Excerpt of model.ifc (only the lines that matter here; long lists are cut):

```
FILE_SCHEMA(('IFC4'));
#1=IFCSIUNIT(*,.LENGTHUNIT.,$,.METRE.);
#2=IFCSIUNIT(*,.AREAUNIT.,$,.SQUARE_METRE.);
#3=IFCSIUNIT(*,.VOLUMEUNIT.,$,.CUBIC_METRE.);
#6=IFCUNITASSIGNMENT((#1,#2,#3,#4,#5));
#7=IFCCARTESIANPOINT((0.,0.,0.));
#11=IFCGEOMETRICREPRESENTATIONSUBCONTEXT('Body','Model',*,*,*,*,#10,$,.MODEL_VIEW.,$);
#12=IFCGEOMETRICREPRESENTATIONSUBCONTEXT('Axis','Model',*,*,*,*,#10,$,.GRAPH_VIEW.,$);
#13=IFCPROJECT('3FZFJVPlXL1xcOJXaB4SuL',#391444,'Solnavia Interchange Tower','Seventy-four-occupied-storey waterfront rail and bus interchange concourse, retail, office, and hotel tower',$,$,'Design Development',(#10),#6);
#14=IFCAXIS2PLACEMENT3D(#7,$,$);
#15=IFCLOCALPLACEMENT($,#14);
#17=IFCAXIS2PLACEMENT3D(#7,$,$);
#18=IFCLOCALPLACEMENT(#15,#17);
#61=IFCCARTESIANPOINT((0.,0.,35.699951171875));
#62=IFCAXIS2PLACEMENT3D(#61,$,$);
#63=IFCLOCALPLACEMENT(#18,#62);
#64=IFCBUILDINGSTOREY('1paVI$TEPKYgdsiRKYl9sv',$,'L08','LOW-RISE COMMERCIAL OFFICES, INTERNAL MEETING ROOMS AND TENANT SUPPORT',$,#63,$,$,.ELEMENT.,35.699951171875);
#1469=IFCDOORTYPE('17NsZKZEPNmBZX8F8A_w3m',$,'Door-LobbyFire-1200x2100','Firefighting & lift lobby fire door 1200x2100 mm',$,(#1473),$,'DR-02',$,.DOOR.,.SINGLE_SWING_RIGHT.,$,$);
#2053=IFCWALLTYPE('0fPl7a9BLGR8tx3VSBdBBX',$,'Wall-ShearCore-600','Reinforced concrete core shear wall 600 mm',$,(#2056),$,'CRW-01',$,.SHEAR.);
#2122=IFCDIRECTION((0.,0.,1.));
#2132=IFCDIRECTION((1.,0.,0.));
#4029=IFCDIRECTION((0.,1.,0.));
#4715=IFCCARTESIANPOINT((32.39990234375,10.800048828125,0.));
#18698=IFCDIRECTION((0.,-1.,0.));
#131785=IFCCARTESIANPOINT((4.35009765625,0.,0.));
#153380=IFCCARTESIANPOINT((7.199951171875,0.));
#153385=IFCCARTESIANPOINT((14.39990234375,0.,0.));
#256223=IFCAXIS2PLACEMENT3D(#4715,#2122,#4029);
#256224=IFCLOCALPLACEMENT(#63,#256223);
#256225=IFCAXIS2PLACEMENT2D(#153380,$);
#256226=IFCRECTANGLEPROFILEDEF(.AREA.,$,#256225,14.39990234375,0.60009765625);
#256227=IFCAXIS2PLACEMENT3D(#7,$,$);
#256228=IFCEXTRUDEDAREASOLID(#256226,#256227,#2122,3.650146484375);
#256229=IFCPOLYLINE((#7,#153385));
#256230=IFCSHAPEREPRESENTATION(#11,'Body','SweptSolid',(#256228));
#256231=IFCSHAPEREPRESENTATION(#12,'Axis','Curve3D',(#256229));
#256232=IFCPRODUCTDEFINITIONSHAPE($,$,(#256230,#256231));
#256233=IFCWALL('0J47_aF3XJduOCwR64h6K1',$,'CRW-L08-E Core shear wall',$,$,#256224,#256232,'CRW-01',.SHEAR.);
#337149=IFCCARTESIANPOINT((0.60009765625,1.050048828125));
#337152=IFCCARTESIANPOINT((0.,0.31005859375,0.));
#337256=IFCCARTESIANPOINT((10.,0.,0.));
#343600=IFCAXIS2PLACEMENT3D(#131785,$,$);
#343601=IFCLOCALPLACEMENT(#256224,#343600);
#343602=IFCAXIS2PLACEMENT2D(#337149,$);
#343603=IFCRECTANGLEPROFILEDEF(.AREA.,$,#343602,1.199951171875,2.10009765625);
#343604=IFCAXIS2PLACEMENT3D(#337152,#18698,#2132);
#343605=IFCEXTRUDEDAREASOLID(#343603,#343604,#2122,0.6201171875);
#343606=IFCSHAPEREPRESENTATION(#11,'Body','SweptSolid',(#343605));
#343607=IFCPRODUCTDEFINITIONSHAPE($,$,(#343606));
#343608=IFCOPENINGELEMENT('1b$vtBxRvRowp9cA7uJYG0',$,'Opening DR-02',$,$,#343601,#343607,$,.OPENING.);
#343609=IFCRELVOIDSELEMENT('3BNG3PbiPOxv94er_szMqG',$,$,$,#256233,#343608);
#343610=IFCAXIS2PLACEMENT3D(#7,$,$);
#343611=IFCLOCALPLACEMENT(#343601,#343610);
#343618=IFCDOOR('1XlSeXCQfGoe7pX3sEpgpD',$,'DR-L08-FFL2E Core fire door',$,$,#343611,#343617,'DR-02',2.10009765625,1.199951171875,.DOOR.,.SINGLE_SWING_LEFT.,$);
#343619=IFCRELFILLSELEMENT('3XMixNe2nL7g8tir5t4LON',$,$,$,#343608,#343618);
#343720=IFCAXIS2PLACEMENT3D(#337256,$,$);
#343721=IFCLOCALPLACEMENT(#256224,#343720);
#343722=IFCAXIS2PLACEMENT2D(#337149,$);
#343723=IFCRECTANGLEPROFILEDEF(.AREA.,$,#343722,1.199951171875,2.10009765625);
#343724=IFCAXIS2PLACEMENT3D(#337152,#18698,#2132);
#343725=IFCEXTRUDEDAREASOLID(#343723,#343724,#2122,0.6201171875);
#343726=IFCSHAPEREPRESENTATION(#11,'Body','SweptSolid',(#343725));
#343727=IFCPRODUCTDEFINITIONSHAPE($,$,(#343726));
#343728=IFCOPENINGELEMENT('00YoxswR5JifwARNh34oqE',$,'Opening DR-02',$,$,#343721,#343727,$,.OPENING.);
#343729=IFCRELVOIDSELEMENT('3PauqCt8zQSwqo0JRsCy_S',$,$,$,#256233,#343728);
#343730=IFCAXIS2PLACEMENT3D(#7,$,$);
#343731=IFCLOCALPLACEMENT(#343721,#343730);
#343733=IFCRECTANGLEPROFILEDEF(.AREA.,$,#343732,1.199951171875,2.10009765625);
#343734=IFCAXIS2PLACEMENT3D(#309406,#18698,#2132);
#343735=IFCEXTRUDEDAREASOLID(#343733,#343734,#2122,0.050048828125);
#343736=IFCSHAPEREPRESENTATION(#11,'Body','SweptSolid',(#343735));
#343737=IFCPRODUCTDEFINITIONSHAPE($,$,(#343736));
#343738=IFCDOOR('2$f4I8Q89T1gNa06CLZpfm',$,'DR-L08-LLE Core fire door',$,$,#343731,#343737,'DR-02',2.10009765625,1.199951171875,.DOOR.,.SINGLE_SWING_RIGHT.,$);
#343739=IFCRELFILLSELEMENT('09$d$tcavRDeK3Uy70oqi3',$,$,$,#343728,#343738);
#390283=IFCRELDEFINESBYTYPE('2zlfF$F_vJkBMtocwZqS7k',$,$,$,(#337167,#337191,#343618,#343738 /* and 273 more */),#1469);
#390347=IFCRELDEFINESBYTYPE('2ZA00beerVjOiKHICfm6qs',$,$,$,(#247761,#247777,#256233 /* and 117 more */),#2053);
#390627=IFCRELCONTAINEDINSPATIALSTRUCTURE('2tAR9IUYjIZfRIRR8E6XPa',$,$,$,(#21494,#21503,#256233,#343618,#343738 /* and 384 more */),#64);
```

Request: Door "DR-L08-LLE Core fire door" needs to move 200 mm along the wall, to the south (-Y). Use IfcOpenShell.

```python
import ifcopenshell
import ifcopenshell.api.geometry
import ifcopenshell.util.placement

model = ifcopenshell.open("model.ifc")

door = model.by_guid("2$f4I8Q89T1gNa06CLZpfm")
opening = door.FillsVoids[0].RelatingOpeningElement
wall = opening.VoidsElements[0].RelatingBuildingElement

wall_matrix = ifcopenshell.util.placement.get_local_placement(wall.ObjectPlacement)
shift = wall_matrix[:3, 0] * -0.2
before = ifcopenshell.util.placement.get_local_placement(door.ObjectPlacement)[:3, 3].copy()

# The door is placed relative to its opening, so it follows when the opening moves.
matrix = ifcopenshell.util.placement.get_local_placement(opening.ObjectPlacement)
matrix[:3, 3] += shift
ifcopenshell.api.geometry.edit_object_placement(
    model, product=opening, matrix=matrix, is_si=False, should_transform_children=True
)

after = ifcopenshell.util.placement.get_local_placement(door.ObjectPlacement)[:3, 3]
print("door moved by", (after - before).round(3) + 0.0)

model.write("model_v2.ifc")
```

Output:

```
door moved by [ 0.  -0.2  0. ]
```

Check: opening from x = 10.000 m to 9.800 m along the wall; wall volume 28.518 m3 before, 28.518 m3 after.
